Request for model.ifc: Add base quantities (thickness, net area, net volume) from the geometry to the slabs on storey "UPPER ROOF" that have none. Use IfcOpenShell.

First a look at what the model holds.

```python
import ifcopenshell
import ifcopenshell.util.element
import ifcopenshell.util.unit

model = ifcopenshell.open("model.ifc")
print(model.schema)
for unit_type in ("LENGTHUNIT", "AREAUNIT", "VOLUMEUNIT"):
    print(unit_type, ifcopenshell.util.unit.calculate_unit_scale(model, unit_type))
storey = next(s for s in model.by_type("IfcBuildingStorey") if s.Name == "UPPER ROOF")
slabs = [e for e in ifcopenshell.util.element.get_decomposition(storey) if e.is_a("IfcSlab")]
for e in sorted(slabs, key=lambda e: e.id()):
    print(e.id(), e.is_a(), e.Name, list(ifcopenshell.util.element.get_psets(e, qtos_only=True)), sep=" | ")
```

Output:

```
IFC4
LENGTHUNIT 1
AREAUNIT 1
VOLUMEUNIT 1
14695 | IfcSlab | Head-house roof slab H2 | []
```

```python
import ifcopenshell
import ifcopenshell.api.pset
import ifcopenshell.geom
import ifcopenshell.util.element
import ifcopenshell.util.shape
import ifcopenshell.util.unit

model = ifcopenshell.open("model.ifc")
unit_scale = ifcopenshell.util.unit.calculate_unit_scale(model)
area_scale = ifcopenshell.util.unit.calculate_unit_scale(model, "AREAUNIT")
volume_scale = ifcopenshell.util.unit.calculate_unit_scale(model, "VOLUMEUNIT")
settings = ifcopenshell.geom.settings()

storey = next(s for s in model.by_type("IfcBuildingStorey") if s.Name == "UPPER ROOF")
slabs = [e for e in ifcopenshell.util.element.get_decomposition(storey) if e.is_a("IfcSlab")]

for e in sorted(slabs, key=lambda e: e.id()):
    if ifcopenshell.util.element.get_psets(e, qtos_only=True, should_inherit=False):
        continue
    # Geometry comes back in metres, in the element's own axes.
    shape = ifcopenshell.geom.create_shape(settings, e)
    values = {
        "Width": ifcopenshell.util.shape.get_z(shape.geometry) / unit_scale,
        "NetArea": ifcopenshell.util.shape.get_footprint_area(shape.geometry) / area_scale,
        "NetVolume": ifcopenshell.util.shape.get_volume(shape.geometry) / volume_scale,
    }
    qto = ifcopenshell.api.pset.add_qto(model, product=e, name="Qto_SlabBaseQuantities")
    ifcopenshell.api.pset.edit_qto(model, qto=qto, properties=values)
    print(e.id(), {k: round(v, 3) for k, v in values.items()})

model.write("model_rev.ifc")
```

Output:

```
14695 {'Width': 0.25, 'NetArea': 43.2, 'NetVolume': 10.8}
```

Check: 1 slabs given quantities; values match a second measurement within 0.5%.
